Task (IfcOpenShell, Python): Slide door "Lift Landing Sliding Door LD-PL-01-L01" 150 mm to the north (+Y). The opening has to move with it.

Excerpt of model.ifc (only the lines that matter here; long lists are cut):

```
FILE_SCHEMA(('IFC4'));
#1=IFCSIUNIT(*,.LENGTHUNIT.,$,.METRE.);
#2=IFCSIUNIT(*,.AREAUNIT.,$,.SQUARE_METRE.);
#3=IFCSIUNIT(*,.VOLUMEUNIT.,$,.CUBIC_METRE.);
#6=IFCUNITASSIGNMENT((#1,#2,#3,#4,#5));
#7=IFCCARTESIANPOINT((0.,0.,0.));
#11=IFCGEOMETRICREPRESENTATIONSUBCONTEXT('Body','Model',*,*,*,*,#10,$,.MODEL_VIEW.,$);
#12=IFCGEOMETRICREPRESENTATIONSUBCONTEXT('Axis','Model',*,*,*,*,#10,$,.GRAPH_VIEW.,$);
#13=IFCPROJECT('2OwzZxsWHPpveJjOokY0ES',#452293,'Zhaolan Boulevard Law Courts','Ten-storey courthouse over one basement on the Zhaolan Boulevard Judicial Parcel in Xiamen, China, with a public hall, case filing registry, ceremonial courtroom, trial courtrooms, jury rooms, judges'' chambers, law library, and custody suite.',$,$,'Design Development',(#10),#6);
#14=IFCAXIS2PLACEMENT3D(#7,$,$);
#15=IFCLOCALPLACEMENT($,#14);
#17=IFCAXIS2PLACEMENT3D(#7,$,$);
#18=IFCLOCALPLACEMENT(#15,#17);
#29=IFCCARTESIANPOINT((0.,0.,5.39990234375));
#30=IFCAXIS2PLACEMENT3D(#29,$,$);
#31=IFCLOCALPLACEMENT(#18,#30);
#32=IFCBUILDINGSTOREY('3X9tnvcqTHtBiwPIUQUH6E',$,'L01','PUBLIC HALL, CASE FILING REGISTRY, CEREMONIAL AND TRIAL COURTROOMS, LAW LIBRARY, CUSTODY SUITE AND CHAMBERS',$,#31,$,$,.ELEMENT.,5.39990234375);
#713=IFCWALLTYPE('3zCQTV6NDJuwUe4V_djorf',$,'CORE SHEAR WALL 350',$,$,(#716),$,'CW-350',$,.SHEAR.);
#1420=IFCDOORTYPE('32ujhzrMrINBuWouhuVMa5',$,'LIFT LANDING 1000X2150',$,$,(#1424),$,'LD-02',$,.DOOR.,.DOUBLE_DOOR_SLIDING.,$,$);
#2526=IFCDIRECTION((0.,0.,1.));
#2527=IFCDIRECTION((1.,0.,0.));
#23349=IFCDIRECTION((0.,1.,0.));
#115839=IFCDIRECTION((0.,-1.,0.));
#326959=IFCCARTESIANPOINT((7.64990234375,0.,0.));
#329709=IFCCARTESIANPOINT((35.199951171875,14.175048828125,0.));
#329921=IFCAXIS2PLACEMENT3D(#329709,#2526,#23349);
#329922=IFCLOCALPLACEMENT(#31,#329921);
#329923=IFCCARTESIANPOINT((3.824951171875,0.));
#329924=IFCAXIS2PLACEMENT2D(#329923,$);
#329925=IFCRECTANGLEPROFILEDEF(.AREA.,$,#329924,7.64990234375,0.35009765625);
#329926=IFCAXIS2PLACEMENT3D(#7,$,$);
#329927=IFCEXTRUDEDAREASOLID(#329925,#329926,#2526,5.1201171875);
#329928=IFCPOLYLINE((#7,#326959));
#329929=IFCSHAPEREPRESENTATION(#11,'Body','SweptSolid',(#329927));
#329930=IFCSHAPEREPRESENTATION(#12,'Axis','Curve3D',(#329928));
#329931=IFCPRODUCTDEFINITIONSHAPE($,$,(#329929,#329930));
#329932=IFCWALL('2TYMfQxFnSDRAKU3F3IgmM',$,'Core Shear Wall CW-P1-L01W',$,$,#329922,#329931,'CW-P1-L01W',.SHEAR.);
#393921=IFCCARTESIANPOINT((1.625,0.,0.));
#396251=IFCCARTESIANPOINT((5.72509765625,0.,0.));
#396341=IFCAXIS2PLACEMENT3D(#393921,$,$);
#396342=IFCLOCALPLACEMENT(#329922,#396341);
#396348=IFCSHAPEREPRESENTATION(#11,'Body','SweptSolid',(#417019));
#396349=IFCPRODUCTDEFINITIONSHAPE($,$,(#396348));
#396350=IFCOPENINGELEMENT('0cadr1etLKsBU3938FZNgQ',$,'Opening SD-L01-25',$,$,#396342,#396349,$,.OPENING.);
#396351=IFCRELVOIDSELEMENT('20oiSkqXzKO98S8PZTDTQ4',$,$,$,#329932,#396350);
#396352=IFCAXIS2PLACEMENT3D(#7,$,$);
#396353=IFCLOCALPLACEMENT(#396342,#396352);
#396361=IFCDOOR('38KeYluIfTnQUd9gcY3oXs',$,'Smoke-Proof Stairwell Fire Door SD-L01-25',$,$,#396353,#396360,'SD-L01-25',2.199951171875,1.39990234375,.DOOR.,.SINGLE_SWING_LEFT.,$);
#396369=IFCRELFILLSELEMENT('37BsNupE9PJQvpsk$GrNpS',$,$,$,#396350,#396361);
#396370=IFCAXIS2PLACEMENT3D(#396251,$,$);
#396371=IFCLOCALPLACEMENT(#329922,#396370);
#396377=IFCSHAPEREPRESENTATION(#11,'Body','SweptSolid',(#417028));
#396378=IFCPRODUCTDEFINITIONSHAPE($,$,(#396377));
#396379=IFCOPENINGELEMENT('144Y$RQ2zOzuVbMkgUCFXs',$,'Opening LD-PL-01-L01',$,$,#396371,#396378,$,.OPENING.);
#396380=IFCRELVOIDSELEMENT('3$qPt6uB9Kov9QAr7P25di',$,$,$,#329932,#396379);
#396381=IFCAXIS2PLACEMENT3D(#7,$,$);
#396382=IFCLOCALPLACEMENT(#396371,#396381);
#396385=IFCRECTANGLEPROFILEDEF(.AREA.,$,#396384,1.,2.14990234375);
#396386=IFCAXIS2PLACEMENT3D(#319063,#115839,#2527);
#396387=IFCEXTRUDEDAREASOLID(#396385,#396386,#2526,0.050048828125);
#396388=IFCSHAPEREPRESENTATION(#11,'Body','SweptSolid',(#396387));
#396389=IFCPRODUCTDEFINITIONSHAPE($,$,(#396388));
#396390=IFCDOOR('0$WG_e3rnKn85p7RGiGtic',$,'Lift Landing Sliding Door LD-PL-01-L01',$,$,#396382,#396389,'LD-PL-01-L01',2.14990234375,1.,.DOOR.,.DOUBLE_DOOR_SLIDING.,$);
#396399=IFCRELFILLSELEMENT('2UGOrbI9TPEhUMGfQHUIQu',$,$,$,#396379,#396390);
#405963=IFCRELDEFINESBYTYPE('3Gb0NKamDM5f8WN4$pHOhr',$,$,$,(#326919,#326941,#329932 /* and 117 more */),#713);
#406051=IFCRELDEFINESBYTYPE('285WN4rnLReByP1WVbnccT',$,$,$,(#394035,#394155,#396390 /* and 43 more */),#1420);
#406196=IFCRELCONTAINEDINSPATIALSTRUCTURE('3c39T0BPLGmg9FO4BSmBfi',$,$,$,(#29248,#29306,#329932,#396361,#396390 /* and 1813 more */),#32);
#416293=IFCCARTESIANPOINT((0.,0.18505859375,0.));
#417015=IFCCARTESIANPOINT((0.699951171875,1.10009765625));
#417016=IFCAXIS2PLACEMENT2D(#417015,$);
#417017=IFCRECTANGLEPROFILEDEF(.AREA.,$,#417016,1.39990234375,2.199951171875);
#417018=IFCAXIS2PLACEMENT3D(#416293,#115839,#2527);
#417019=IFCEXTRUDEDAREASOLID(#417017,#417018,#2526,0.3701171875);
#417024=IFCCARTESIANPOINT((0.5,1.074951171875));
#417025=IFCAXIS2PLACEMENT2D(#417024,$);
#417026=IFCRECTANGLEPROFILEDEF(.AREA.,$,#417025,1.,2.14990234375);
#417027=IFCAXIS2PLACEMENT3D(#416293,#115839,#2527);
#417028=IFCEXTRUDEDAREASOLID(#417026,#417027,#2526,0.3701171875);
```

```python
import ifcopenshell
import ifcopenshell.api.geometry
import ifcopenshell.util.placement
import ifcopenshell.util.unit

model = ifcopenshell.open("model.ifc")
unit_scale = ifcopenshell.util.unit.calculate_unit_scale(model)

door = model.by_guid("0$WG_e3rnKn85p7RGiGtic")
opening = door.FillsVoids[0].RelatingOpeningElement
wall = opening.VoidsElements[0].RelatingBuildingElement

wall_matrix = ifcopenshell.util.placement.get_local_placement(wall.ObjectPlacement)
shift = wall_matrix[:3, 0] * 0.15 / unit_scale
before = ifcopenshell.util.placement.get_local_placement(door.ObjectPlacement)[:3, 3].copy()

# The door is placed relative to its opening, so it follows when the opening moves.
matrix = ifcopenshell.util.placement.get_local_placement(opening.ObjectPlacement)
matrix[:3, 3] += shift
ifcopenshell.api.geometry.edit_object_placement(
    model, product=opening, matrix=matrix, is_si=False, should_transform_children=True
)

after = ifcopenshell.util.placement.get_local_placement(door.ObjectPlacement)[:3, 3]
print("door moved by", (after - before).round(3) + 0.0)

model.write("model_rev.ifc")
```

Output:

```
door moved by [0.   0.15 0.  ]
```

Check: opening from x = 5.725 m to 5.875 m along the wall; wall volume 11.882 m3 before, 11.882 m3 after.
